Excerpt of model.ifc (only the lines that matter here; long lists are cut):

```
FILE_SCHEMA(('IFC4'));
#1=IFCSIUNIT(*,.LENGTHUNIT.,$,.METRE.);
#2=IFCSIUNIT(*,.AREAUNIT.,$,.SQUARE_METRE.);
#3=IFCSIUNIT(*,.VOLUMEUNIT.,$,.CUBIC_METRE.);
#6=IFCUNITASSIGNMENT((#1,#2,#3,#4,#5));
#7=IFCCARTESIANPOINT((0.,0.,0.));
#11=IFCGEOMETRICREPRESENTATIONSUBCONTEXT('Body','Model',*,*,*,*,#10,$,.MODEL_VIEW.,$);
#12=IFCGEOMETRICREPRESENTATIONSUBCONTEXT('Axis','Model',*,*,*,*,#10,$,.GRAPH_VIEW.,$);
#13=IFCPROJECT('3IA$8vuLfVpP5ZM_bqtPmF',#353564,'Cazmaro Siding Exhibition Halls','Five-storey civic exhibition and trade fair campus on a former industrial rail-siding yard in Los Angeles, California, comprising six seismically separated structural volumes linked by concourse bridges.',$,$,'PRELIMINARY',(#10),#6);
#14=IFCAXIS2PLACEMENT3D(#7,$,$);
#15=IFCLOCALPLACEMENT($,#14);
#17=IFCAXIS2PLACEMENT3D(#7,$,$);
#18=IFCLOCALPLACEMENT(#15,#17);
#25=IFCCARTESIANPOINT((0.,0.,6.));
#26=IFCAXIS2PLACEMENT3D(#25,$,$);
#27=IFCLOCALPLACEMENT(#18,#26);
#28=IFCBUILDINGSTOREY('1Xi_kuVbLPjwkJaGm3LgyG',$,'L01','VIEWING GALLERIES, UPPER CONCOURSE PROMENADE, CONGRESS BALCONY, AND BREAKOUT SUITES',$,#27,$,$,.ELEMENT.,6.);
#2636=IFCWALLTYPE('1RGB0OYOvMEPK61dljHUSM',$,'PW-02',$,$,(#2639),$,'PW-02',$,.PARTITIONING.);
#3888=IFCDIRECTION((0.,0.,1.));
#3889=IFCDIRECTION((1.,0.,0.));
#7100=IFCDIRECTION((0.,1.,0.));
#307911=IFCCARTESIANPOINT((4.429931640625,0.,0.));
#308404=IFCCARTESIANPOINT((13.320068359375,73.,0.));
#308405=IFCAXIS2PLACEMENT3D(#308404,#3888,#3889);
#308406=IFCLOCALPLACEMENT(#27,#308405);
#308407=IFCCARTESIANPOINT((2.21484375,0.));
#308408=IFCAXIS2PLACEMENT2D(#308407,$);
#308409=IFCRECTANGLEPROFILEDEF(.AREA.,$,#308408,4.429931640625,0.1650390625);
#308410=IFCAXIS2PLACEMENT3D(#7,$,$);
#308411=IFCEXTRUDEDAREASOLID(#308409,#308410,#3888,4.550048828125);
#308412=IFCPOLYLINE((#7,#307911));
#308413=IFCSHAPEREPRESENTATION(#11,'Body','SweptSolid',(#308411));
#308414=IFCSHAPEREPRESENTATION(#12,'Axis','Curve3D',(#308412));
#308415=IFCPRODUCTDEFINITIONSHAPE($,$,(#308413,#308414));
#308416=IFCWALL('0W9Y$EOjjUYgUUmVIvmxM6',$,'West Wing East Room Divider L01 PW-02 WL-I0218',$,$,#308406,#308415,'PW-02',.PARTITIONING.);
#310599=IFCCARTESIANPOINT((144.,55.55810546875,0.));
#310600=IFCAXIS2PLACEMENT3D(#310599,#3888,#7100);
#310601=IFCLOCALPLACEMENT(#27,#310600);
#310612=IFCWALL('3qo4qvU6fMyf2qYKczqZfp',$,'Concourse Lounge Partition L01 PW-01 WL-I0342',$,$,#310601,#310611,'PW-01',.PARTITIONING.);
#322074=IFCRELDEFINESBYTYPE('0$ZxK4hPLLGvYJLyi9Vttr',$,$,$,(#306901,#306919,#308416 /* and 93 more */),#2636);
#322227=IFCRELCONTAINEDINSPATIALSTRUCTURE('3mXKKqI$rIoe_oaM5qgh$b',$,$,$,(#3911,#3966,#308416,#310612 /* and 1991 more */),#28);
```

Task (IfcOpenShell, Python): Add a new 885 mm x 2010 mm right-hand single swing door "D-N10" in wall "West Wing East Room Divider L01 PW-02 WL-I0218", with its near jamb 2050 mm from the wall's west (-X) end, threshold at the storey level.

```python
import numpy as np
import ifcopenshell
import ifcopenshell.api.feature
import ifcopenshell.api.geometry
import ifcopenshell.api.root
import ifcopenshell.api.spatial
import ifcopenshell.geom
import ifcopenshell.util.element
import ifcopenshell.util.placement
import ifcopenshell.util.representation
import ifcopenshell.util.shape
import ifcopenshell.util.unit

model = ifcopenshell.open("model.ifc")
unit_scale = ifcopenshell.util.unit.calculate_unit_scale(model)
settings = ifcopenshell.geom.settings()


def volume(element):
    """Net volume in cubic metres, openings subtracted."""
    shape = ifcopenshell.geom.create_shape(settings, element)
    return ifcopenshell.util.shape.get_volume(shape.geometry)


wall = model.by_guid("0W9Y$EOjjUYgUUmVIvmxM6")
storey = ifcopenshell.util.element.get_container(wall, ifc_class="IfcBuildingStorey")
context = ifcopenshell.util.representation.get_context(model, "Model", "Body", "MODEL_VIEW")
before = volume(wall)

width, height, from_end, sill = 0.885, 2.01, 2.05, 0.0  # metres

# The wall runs along its own X axis, and the end named is its -X end.
wall_shape = ifcopenshell.geom.create_shape(settings, wall)
x, y, z = ifcopenshell.util.shape.get_vertices(wall_shape.geometry).T
start = x.min() + from_end
face, thickness = float(y.min()), float(y.max() - y.min())
wall_matrix = ifcopenshell.util.placement.get_local_placement(wall.ObjectPlacement)
level = ifcopenshell.util.placement.get_local_placement(storey.ObjectPlacement)[2, 3]


def in_wall(x, y):
    """Placement at x, y metres in the wall's axes, at sill height."""
    matrix = wall_matrix.copy()
    matrix[:, 3] = wall_matrix @ np.array([x / unit_scale, y / unit_scale, 0.0, 1.0])
    matrix[2, 3] = level + sill / unit_scale
    return matrix


# Opening: a box that overshoots both wall faces by 50 mm.
opening = ifcopenshell.api.root.create_entity(model, ifc_class="IfcOpeningElement", predefined_type="OPENING")
box = ifcopenshell.api.geometry.add_wall_representation(
    model, context=context, length=width, height=height, thickness=thickness + 0.1
)
ifcopenshell.api.geometry.assign_representation(model, product=opening, representation=box)
ifcopenshell.api.geometry.edit_object_placement(model, product=opening, matrix=in_wall(start, face - 0.05), is_si=False)
ifcopenshell.api.feature.add_feature(model, feature=opening, element=wall)

door = ifcopenshell.api.root.create_entity(model, ifc_class="IfcDoor", name="D-N10", predefined_type="DOOR")
door.OverallWidth, door.OverallHeight = width / unit_scale, height / unit_scale
door.OperationType = "SINGLE_SWING_RIGHT"
body = ifcopenshell.api.geometry.add_door_representation(
    model,
    context=context,
    overall_width=door.OverallWidth,
    overall_height=door.OverallHeight,
    operation_type="SINGLE_SWING_RIGHT",
    lining_properties={"LiningDepth": thickness / unit_scale, "ThresholdDepth": thickness / unit_scale},
)
ifcopenshell.api.geometry.assign_representation(model, product=door, representation=body)
ifcopenshell.api.spatial.assign_container(model, products=[door], relating_structure=storey)
ifcopenshell.api.feature.add_filling(model, opening=opening, element=door)

# The lining spans the wall, so the door starts at the wall face.
ifcopenshell.api.geometry.edit_object_placement(model, product=door, matrix=in_wall(start, face), is_si=False)

after = volume(wall)

print(f"wall volume {before:.3f} -> {after:.3f} m3")

model.write("model_updated.ifc")
```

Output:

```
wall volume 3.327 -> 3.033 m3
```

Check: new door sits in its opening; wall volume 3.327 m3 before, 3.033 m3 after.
